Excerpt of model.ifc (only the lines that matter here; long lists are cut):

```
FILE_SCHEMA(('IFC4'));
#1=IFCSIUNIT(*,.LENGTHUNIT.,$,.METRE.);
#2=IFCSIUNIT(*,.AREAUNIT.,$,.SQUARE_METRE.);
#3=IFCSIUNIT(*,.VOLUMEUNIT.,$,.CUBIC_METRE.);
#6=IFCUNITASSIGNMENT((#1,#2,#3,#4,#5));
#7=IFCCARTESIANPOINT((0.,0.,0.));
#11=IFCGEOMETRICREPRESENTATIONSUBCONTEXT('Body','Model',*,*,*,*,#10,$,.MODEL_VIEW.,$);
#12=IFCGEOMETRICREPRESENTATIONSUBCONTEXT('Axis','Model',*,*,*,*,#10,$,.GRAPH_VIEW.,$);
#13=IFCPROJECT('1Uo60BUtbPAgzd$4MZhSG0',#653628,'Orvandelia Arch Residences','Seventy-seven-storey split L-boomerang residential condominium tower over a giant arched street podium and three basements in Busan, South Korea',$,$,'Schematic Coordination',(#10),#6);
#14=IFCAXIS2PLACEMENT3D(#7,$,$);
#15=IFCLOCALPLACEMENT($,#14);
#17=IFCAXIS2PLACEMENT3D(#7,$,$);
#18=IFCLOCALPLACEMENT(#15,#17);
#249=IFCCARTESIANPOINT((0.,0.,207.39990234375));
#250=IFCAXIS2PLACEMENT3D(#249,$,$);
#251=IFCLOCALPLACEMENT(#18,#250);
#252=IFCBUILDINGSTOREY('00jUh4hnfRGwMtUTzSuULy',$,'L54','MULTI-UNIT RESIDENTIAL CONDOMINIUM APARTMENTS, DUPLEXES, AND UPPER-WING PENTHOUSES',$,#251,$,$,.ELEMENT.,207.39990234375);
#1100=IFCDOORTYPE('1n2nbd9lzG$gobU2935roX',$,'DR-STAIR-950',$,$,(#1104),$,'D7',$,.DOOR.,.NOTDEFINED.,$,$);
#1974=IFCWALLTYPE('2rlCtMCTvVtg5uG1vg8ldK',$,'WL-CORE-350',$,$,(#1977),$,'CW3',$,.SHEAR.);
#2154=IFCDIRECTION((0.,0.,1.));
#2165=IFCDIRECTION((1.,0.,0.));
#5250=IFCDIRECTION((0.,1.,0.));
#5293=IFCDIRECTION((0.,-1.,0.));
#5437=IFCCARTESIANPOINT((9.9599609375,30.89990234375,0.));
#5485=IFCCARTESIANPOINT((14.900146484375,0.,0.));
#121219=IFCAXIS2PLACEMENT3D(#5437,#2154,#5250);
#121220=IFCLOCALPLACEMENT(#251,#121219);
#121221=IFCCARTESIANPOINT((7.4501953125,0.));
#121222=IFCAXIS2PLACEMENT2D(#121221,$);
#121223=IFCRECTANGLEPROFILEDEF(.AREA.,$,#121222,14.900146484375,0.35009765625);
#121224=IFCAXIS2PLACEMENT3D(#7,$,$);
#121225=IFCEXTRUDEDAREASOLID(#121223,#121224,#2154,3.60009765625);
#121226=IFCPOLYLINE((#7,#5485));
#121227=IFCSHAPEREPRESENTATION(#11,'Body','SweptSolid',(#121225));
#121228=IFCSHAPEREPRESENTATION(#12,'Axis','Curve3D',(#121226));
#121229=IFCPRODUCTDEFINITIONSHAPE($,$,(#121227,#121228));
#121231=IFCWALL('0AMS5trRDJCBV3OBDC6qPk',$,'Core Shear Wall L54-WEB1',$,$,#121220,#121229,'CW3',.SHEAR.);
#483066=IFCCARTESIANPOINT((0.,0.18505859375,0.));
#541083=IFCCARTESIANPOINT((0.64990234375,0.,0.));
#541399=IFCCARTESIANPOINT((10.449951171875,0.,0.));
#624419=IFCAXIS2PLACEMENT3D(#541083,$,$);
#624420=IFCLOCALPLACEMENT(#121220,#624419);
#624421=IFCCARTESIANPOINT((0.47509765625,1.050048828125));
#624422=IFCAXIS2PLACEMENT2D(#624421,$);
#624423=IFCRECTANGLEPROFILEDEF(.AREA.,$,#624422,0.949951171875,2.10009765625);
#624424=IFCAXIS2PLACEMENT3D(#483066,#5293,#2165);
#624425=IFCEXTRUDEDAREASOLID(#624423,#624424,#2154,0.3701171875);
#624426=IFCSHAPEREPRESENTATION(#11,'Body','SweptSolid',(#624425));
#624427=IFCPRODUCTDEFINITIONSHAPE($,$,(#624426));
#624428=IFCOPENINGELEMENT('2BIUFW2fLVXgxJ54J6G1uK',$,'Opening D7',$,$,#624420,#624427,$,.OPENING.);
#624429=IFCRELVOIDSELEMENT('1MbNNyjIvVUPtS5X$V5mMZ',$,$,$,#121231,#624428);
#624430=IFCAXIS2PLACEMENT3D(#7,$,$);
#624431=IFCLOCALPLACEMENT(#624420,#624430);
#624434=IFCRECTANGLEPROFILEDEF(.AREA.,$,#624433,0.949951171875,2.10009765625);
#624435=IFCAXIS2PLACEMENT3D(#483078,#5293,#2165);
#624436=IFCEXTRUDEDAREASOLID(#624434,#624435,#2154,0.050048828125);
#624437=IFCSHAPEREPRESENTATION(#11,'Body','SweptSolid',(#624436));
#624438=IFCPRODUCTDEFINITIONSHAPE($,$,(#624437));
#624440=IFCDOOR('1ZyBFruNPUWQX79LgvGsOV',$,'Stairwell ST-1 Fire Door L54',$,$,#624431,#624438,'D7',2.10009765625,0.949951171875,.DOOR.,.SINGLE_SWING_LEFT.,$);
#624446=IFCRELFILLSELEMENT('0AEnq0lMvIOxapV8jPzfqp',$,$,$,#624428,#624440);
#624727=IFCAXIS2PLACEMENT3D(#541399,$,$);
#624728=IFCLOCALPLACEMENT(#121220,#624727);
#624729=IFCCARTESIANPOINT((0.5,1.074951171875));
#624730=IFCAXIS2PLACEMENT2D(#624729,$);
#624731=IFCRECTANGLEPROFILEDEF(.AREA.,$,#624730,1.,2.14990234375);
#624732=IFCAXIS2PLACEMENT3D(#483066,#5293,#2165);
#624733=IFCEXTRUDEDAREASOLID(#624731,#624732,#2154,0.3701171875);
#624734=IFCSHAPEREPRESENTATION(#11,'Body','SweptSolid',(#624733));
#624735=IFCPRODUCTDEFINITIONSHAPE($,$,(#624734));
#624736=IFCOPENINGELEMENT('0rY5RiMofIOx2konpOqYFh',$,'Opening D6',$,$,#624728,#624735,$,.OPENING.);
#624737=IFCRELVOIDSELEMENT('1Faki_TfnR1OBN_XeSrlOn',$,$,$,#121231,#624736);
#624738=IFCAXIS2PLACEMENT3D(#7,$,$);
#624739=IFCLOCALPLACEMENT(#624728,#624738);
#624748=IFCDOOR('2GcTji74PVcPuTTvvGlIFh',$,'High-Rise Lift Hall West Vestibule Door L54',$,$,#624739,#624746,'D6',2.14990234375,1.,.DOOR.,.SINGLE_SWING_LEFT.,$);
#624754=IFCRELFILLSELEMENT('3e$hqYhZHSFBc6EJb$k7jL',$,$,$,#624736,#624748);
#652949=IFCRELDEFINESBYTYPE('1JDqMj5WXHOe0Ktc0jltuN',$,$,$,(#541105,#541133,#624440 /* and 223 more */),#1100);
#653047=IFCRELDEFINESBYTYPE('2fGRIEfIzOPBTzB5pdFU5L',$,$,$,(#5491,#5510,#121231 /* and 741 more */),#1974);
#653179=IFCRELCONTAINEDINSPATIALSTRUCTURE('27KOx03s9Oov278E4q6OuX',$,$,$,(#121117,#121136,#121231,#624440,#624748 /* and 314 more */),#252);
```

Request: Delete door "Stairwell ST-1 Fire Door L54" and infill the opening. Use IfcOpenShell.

```python
import ifcopenshell
import ifcopenshell.api.feature
import ifcopenshell.api.root
import ifcopenshell.geom
import ifcopenshell.util.shape

model = ifcopenshell.open("model.ifc")
settings = ifcopenshell.geom.settings()


def volume(element):
    """Net volume in cubic metres, openings subtracted."""
    shape = ifcopenshell.geom.create_shape(settings, element)
    return ifcopenshell.util.shape.get_volume(shape.geometry)


door = model.by_guid("1ZyBFruNPUWQX79LgvGsOV")
opening = door.FillsVoids[0].RelatingOpeningElement
wall = opening.VoidsElements[0].RelatingBuildingElement
before = volume(wall)

ifcopenshell.api.root.remove_product(model, product=door)
ifcopenshell.api.feature.remove_feature(model, feature=opening)

after = volume(wall)

print(f"wall volume {before:.3f} -> {after:.3f} m3")

model.write("model_edited.ifc")
```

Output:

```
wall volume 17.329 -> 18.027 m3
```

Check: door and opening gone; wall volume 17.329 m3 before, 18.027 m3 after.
